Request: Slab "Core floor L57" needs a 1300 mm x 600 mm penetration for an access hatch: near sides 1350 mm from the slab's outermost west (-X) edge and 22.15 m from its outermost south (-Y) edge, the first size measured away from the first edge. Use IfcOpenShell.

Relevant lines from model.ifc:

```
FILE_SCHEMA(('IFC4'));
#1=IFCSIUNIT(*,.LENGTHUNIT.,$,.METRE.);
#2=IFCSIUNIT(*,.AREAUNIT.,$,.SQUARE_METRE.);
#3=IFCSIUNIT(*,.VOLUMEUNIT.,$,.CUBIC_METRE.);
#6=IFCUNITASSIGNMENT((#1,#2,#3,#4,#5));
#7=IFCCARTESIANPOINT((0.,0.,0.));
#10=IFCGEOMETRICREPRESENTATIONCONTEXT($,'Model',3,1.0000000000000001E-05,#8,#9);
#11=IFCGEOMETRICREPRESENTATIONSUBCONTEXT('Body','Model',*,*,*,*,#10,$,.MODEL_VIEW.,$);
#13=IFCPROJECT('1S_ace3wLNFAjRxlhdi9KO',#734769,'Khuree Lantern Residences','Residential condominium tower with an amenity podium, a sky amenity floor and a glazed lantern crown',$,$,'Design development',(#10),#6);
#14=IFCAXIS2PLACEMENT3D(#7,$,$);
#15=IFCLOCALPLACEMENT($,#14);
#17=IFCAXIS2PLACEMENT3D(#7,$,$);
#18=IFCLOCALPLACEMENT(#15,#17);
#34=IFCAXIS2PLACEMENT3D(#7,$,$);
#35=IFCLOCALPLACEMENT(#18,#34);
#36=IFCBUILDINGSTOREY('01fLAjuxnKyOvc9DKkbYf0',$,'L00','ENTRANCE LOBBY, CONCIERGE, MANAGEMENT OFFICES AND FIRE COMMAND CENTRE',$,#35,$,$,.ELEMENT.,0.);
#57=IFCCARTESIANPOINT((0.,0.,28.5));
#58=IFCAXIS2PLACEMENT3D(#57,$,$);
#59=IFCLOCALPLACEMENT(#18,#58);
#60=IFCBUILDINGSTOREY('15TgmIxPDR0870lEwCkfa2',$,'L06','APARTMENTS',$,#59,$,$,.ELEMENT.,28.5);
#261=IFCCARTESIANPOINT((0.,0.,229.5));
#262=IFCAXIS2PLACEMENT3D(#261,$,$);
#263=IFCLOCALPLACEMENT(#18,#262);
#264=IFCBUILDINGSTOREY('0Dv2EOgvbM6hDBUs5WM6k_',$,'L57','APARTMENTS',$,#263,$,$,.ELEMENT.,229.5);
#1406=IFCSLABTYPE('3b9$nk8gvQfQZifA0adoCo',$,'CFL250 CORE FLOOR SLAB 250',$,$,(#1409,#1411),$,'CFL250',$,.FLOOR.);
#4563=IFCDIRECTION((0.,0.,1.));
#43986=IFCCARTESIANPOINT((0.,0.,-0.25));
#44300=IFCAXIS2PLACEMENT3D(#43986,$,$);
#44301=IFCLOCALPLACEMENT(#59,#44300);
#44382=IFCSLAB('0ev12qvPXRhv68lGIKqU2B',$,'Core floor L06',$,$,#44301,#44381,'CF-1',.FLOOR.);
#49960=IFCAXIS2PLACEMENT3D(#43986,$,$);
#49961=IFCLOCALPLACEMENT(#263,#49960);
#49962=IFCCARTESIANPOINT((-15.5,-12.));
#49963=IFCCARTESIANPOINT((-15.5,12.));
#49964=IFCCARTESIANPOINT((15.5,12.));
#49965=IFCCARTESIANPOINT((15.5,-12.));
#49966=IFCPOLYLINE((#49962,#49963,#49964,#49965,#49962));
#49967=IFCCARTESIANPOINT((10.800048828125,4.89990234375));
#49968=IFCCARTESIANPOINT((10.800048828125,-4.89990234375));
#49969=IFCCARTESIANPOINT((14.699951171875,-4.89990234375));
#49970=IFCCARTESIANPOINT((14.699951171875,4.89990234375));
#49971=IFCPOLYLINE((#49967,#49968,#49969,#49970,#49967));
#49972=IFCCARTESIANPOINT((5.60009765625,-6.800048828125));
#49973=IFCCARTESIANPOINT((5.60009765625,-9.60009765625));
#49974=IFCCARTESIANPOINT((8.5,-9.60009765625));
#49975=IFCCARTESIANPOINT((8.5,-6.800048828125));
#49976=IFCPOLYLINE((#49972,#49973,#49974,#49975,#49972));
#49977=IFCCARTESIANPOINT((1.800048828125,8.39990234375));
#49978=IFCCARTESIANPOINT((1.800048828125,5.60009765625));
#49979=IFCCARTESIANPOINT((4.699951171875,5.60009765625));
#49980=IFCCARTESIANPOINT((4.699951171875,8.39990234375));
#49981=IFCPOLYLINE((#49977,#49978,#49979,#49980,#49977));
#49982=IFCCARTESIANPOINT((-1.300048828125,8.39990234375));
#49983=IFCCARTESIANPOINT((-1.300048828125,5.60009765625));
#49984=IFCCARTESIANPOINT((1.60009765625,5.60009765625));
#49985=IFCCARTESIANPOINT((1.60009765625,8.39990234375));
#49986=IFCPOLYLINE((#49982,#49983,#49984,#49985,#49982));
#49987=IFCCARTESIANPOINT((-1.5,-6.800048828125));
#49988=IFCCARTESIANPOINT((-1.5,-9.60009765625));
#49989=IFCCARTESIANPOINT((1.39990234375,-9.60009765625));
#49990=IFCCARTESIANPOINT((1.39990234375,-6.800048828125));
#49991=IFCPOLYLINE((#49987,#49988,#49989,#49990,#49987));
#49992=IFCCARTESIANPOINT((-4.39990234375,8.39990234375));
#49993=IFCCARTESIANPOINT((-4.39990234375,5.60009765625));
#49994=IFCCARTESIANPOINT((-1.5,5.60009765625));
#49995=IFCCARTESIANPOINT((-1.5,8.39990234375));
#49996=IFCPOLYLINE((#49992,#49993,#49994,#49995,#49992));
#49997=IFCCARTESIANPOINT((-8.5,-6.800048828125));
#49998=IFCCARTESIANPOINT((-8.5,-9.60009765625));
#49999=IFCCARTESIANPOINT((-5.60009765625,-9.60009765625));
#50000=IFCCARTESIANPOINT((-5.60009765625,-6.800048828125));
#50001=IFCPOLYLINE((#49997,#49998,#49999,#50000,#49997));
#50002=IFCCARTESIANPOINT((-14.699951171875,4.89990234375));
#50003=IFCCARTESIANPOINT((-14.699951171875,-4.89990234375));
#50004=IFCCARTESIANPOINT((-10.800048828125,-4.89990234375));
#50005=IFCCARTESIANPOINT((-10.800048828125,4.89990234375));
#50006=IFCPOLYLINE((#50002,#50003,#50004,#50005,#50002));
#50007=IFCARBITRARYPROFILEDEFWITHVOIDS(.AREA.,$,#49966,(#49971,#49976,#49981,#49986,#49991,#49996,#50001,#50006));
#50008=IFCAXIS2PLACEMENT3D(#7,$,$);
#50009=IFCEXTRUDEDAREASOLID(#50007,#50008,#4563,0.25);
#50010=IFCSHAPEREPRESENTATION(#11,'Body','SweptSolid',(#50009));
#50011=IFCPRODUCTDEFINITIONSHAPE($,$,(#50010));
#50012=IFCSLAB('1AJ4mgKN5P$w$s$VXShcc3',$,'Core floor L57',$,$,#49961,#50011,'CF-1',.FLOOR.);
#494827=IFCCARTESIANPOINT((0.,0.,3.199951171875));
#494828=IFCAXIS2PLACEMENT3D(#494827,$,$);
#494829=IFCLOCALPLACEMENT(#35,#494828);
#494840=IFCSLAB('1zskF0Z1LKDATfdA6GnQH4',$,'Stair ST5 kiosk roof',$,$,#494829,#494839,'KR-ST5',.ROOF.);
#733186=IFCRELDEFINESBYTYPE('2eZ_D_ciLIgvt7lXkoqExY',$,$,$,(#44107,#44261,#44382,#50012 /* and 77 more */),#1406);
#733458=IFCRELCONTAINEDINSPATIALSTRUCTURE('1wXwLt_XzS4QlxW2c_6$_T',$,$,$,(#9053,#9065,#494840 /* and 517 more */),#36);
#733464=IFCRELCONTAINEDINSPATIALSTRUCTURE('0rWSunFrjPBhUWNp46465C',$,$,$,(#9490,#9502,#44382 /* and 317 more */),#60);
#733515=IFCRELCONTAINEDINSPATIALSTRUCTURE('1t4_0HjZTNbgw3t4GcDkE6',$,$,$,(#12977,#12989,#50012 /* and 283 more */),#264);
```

```python
import numpy as np
import ifcopenshell
import ifcopenshell.api.feature
import ifcopenshell.api.geometry
import ifcopenshell.api.root
import ifcopenshell.geom
import ifcopenshell.util.placement
import ifcopenshell.util.representation
import ifcopenshell.util.shape
import ifcopenshell.util.unit

model = ifcopenshell.open("model.ifc")
unit_scale = ifcopenshell.util.unit.calculate_unit_scale(model)
settings = ifcopenshell.geom.settings()


def volume(element):
    """Net volume in cubic metres, openings subtracted."""
    shape = ifcopenshell.geom.create_shape(settings, element)
    return ifcopenshell.util.shape.get_volume(shape.geometry)


slab = model.by_guid("1AJ4mgKN5P$w$s$VXShcc3")
before = volume(slab)

# Extent in the slab's own axes, in metres. The edges named are its -X and -Y sides.
slab_shape = ifcopenshell.geom.create_shape(settings, slab)
vertices = ifcopenshell.util.shape.get_vertices(slab_shape.geometry)
x_min, y_min, bottom = vertices.min(axis=0)
top = vertices[:, 2].max()

opening = ifcopenshell.api.root.create_entity(model, ifc_class="IfcOpeningElement", name="Access hatch opening", predefined_type="OPENING")
context = ifcopenshell.util.representation.get_context(model, "Model", "Body", "MODEL_VIEW")
width, depth = 1.3, 0.6
outline = [(0.0, 0.0), (width, 0.0), (width, depth), (0.0, depth), (0.0, 0.0)]
# Overshoot both faces by 50 mm so the cut is clean.
shape = ifcopenshell.api.geometry.add_slab_representation(
    model, context=context, depth=top - bottom + 0.1, polyline=outline
)
ifcopenshell.api.geometry.assign_representation(model, product=opening, representation=shape)

matrix = ifcopenshell.util.placement.get_local_placement(slab.ObjectPlacement)
matrix[:, 3] = matrix @ np.append(np.array([x_min + 1.35, y_min + 22.15, bottom - 0.05]) / unit_scale, 1.0)
ifcopenshell.api.geometry.edit_object_placement(model, product=opening, matrix=matrix, is_si=False)
ifcopenshell.api.feature.add_feature(model, feature=opening, element=slab)

after = volume(slab)

print(f"slab volume {before:.3f} -> {after:.3f} m3")

model.write("model_edited.ifc")
```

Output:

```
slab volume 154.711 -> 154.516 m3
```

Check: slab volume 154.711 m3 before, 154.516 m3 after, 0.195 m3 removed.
